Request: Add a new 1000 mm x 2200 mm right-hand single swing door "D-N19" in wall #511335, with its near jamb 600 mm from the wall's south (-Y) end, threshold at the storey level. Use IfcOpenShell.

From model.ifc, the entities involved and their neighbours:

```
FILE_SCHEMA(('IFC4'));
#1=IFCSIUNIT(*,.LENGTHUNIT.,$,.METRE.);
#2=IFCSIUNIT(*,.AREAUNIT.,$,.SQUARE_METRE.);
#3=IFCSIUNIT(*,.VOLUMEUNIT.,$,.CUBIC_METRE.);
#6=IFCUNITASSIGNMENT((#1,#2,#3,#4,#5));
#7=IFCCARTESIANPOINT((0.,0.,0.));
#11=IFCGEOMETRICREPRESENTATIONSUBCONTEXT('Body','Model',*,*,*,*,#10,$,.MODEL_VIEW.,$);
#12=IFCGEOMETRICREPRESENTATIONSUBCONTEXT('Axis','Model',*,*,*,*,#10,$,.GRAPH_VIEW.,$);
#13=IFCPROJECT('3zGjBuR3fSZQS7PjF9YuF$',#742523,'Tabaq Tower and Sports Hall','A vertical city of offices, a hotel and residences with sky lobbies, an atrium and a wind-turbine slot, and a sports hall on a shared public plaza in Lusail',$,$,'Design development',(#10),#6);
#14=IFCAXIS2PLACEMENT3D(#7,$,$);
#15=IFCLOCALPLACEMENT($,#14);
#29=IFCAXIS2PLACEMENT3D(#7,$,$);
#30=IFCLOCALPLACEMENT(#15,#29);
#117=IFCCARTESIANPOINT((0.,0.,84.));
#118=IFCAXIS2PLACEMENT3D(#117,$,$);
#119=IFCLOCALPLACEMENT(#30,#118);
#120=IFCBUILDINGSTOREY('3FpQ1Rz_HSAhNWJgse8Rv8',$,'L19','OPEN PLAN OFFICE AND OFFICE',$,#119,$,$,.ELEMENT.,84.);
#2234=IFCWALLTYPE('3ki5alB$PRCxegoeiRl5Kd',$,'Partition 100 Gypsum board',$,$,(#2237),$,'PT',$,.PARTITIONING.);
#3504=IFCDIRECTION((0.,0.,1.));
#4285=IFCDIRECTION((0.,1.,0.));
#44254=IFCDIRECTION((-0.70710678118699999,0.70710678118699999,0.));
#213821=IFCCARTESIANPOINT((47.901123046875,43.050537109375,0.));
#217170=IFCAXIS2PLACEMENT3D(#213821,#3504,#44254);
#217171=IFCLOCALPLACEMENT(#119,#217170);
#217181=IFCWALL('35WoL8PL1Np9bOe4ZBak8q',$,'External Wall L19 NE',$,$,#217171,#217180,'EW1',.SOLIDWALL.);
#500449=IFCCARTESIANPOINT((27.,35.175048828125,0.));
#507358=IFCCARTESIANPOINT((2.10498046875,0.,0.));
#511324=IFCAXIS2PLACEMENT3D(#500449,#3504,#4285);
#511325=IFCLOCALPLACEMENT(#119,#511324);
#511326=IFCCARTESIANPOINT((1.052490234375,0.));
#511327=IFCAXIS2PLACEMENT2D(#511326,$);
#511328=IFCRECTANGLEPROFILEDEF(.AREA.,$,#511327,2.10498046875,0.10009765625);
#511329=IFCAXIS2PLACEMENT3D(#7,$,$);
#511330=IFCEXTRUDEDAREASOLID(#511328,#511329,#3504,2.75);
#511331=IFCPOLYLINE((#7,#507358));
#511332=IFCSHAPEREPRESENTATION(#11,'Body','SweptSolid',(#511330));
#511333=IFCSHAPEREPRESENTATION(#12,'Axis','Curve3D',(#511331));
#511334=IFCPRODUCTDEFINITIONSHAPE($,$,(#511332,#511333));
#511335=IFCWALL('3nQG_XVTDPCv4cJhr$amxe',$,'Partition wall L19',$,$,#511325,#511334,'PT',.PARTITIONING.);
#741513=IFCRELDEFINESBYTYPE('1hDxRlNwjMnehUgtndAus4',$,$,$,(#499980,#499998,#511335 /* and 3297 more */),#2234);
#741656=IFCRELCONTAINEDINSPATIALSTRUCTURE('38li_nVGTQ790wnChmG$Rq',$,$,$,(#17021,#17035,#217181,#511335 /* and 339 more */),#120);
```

```python
import numpy as np
import ifcopenshell
import ifcopenshell.api.feature
import ifcopenshell.api.geometry
import ifcopenshell.api.root
import ifcopenshell.api.spatial
import ifcopenshell.geom
import ifcopenshell.util.element
import ifcopenshell.util.placement
import ifcopenshell.util.representation
import ifcopenshell.util.shape
import ifcopenshell.util.unit

model = ifcopenshell.open("model.ifc")
unit_scale = ifcopenshell.util.unit.calculate_unit_scale(model)
settings = ifcopenshell.geom.settings()


def volume(element):
    """Net volume in cubic metres, openings subtracted."""
    shape = ifcopenshell.geom.create_shape(settings, element)
    return ifcopenshell.util.shape.get_volume(shape.geometry)


wall = model.by_guid("3nQG_XVTDPCv4cJhr$amxe")
storey = ifcopenshell.util.element.get_container(wall, ifc_class="IfcBuildingStorey")
context = ifcopenshell.util.representation.get_context(model, "Model", "Body", "MODEL_VIEW")
before = volume(wall)

width, height, from_end, sill = 1, 2.2, 0.6, 0.0  # metres

# The wall runs along its own X axis, and the end named is its -X end.
wall_shape = ifcopenshell.geom.create_shape(settings, wall)
x, y, z = ifcopenshell.util.shape.get_vertices(wall_shape.geometry).T
start = x.min() + from_end
face, thickness = float(y.min()), float(y.max() - y.min())
wall_matrix = ifcopenshell.util.placement.get_local_placement(wall.ObjectPlacement)
level = ifcopenshell.util.placement.get_local_placement(storey.ObjectPlacement)[2, 3]


def in_wall(x, y):
    """Placement at x, y metres in the wall's axes, at sill height."""
    matrix = wall_matrix.copy()
    matrix[:, 3] = wall_matrix @ np.array([x / unit_scale, y / unit_scale, 0.0, 1.0])
    matrix[2, 3] = level + sill / unit_scale
    return matrix


# Opening: a box that overshoots both wall faces by 50 mm.
opening = ifcopenshell.api.root.create_entity(model, ifc_class="IfcOpeningElement", predefined_type="OPENING")
box = ifcopenshell.api.geometry.add_wall_representation(
    model, context=context, length=width, height=height, thickness=thickness + 0.1
)
ifcopenshell.api.geometry.assign_representation(model, product=opening, representation=box)
ifcopenshell.api.geometry.edit_object_placement(model, product=opening, matrix=in_wall(start, face - 0.05), is_si=False)
ifcopenshell.api.feature.add_feature(model, feature=opening, element=wall)

door = ifcopenshell.api.root.create_entity(model, ifc_class="IfcDoor", name="D-N19", predefined_type="DOOR")
door.OverallWidth, door.OverallHeight = width / unit_scale, height / unit_scale
door.OperationType = "SINGLE_SWING_RIGHT"
body = ifcopenshell.api.geometry.add_door_representation(
    model,
    context=context,
    overall_width=door.OverallWidth,
    overall_height=door.OverallHeight,
    operation_type="SINGLE_SWING_RIGHT",
    lining_properties={"LiningDepth": thickness / unit_scale, "ThresholdDepth": thickness / unit_scale},
)
ifcopenshell.api.geometry.assign_representation(model, product=door, representation=body)
ifcopenshell.api.spatial.assign_container(model, products=[door], relating_structure=storey)
ifcopenshell.api.feature.add_filling(model, opening=opening, element=door)

# The lining spans the wall, so the door starts at the wall face.
ifcopenshell.api.geometry.edit_object_placement(model, product=door, matrix=in_wall(start, face), is_si=False)

after = volume(wall)

print(f"wall volume {before:.3f} -> {after:.3f} m3")

model.write("model_v2.ifc")
```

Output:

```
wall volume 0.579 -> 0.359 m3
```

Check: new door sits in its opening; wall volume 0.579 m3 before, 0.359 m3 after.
